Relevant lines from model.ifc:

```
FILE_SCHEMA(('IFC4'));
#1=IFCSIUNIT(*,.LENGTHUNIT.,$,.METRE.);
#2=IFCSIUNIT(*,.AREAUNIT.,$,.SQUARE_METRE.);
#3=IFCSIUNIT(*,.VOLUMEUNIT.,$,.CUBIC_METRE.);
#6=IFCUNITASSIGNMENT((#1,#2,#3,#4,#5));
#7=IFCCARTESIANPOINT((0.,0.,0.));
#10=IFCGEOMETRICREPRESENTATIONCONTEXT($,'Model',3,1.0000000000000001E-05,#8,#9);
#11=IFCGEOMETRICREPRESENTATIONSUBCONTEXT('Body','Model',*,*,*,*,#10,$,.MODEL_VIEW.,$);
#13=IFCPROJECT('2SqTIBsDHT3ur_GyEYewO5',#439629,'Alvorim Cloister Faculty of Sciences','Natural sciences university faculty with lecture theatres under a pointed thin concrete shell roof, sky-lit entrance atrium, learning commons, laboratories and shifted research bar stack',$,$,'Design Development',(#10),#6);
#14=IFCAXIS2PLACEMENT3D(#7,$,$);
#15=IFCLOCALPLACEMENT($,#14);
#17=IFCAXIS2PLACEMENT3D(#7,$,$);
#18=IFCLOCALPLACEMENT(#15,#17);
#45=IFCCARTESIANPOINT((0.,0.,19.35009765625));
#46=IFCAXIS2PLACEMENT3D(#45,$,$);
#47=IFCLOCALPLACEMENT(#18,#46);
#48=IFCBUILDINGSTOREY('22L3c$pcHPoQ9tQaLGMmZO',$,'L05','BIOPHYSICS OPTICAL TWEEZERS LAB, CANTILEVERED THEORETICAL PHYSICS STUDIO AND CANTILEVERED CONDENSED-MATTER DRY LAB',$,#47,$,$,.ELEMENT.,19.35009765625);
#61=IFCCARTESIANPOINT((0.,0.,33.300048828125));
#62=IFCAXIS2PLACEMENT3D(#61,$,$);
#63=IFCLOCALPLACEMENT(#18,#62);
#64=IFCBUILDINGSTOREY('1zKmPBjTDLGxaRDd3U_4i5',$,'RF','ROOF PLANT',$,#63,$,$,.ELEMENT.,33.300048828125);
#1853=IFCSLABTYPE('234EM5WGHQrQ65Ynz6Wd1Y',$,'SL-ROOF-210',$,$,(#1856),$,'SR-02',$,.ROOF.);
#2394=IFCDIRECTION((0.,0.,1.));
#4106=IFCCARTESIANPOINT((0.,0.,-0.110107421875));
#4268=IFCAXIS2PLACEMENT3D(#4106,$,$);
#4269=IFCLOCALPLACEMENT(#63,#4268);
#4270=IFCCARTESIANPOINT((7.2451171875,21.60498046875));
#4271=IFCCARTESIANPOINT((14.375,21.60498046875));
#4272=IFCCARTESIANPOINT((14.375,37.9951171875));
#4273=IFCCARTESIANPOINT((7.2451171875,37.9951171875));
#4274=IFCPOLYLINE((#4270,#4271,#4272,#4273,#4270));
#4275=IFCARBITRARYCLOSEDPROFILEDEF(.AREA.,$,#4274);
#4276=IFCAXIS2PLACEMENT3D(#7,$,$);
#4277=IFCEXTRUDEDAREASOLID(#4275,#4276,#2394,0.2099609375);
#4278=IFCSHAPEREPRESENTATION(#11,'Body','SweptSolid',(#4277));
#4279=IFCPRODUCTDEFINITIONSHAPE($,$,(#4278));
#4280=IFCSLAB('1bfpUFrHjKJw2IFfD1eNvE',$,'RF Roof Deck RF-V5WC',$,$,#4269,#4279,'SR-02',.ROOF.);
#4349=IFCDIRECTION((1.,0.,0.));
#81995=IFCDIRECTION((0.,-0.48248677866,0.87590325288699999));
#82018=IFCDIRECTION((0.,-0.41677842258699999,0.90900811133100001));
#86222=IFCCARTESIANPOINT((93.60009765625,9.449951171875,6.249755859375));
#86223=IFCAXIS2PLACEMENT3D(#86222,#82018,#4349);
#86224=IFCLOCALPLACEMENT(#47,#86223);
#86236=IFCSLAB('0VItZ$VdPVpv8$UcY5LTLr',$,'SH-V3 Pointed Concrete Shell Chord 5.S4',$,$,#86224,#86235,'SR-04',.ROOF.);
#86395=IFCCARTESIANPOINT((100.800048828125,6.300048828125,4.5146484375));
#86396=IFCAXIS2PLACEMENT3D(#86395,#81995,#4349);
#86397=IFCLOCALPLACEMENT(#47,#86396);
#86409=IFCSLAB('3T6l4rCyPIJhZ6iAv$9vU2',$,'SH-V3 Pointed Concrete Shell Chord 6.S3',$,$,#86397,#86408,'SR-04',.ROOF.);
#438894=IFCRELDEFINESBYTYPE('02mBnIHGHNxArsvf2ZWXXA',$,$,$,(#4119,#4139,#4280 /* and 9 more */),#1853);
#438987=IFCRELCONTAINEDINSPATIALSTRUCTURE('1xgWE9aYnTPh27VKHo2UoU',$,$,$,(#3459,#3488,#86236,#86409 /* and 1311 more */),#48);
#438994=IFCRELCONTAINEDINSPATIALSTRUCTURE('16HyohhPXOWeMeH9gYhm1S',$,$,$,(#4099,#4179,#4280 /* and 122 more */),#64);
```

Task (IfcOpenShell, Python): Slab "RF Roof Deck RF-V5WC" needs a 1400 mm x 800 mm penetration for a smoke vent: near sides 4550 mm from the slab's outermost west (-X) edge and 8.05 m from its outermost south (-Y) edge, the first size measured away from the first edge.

```python
import numpy as np
import ifcopenshell
import ifcopenshell.api.feature
import ifcopenshell.api.geometry
import ifcopenshell.api.root
import ifcopenshell.geom
import ifcopenshell.util.placement
import ifcopenshell.util.representation
import ifcopenshell.util.shape
import ifcopenshell.util.unit

model = ifcopenshell.open("model.ifc")
unit_scale = ifcopenshell.util.unit.calculate_unit_scale(model)
settings = ifcopenshell.geom.settings()


def volume(element):
    """Net volume in cubic metres, openings subtracted."""
    shape = ifcopenshell.geom.create_shape(settings, element)
    return ifcopenshell.util.shape.get_volume(shape.geometry)


slab = model.by_guid("1bfpUFrHjKJw2IFfD1eNvE")
before = volume(slab)

# Extent in the slab's own axes, in metres. The edges named are its -X and -Y sides.
slab_shape = ifcopenshell.geom.create_shape(settings, slab)
vertices = ifcopenshell.util.shape.get_vertices(slab_shape.geometry)
x_min, y_min, bottom = vertices.min(axis=0)
top = vertices[:, 2].max()

opening = ifcopenshell.api.root.create_entity(model, ifc_class="IfcOpeningElement", name="Smoke vent opening", predefined_type="OPENING")
context = ifcopenshell.util.representation.get_context(model, "Model", "Body", "MODEL_VIEW")
width, depth = 1.4, 0.8
outline = [(0.0, 0.0), (width, 0.0), (width, depth), (0.0, depth), (0.0, 0.0)]
# Overshoot both faces by 50 mm so the cut is clean.
shape = ifcopenshell.api.geometry.add_slab_representation(
    model, context=context, depth=top - bottom + 0.1, polyline=outline
)
ifcopenshell.api.geometry.assign_representation(model, product=opening, representation=shape)

matrix = ifcopenshell.util.placement.get_local_placement(slab.ObjectPlacement)
matrix[:, 3] = matrix @ np.append(np.array([x_min + 4.55, y_min + 8.05, bottom - 0.05]) / unit_scale, 1.0)
ifcopenshell.api.geometry.edit_object_placement(model, product=opening, matrix=matrix, is_si=False)
ifcopenshell.api.feature.add_feature(model, feature=opening, element=slab)

after = volume(slab)

print(f"slab volume {before:.3f} -> {after:.3f} m3")

model.write("model_v2.ifc")
```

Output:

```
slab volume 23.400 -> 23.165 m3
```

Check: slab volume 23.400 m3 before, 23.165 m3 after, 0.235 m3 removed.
